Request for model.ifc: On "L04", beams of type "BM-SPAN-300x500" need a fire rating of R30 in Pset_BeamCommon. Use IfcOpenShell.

First a look at what the model holds.

```python
import ifcopenshell
import ifcopenshell.util.element

model = ifcopenshell.open("model.ifc")
print(model.schema)
storey = next(s for s in model.by_type("IfcBuildingStorey") if s.Name == "L04")
beams = [e for e in ifcopenshell.util.element.get_decomposition(storey) if e.is_a("IfcBeam")]
seen = {}
for e in beams:
    element_type = ifcopenshell.util.element.get_type(e)
    key = (element_type.Name if element_type != e and element_type else None, ifcopenshell.util.element.get_pset(e, "Pset_BeamCommon", "FireRating"))
    seen[key] = seen.get(key, 0) + 1
for (name, value), count in sorted(seen.items(), key=str):
    print(count, "x", name, "|", value)
```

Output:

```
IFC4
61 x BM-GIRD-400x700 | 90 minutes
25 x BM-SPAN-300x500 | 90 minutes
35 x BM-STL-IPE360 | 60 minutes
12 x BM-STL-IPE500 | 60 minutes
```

```python
import ifcopenshell
import ifcopenshell.api.pset
import ifcopenshell.util.element

model = ifcopenshell.open("model.ifc")

storey = next(s for s in model.by_type("IfcBuildingStorey") if s.Name == "L04")
beams = [e for e in ifcopenshell.util.element.get_decomposition(storey) if e.is_a("IfcBeam")]

count = 0
for e in beams:
    element_type = ifcopenshell.util.element.get_type(e)
    if element_type in (None, e) or element_type.Name != "BM-SPAN-300x500":
        continue
    # add_pset returns the element's existing set when there is one.
    pset = ifcopenshell.api.pset.add_pset(model, product=e, name="Pset_BeamCommon")
    ifcopenshell.api.pset.edit_pset(model, pset=pset, properties={"FireRating": "R30"})
    count += 1

print(count, "beams updated")

model.write("model_v2.ifc")
```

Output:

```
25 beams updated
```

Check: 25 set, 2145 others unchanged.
